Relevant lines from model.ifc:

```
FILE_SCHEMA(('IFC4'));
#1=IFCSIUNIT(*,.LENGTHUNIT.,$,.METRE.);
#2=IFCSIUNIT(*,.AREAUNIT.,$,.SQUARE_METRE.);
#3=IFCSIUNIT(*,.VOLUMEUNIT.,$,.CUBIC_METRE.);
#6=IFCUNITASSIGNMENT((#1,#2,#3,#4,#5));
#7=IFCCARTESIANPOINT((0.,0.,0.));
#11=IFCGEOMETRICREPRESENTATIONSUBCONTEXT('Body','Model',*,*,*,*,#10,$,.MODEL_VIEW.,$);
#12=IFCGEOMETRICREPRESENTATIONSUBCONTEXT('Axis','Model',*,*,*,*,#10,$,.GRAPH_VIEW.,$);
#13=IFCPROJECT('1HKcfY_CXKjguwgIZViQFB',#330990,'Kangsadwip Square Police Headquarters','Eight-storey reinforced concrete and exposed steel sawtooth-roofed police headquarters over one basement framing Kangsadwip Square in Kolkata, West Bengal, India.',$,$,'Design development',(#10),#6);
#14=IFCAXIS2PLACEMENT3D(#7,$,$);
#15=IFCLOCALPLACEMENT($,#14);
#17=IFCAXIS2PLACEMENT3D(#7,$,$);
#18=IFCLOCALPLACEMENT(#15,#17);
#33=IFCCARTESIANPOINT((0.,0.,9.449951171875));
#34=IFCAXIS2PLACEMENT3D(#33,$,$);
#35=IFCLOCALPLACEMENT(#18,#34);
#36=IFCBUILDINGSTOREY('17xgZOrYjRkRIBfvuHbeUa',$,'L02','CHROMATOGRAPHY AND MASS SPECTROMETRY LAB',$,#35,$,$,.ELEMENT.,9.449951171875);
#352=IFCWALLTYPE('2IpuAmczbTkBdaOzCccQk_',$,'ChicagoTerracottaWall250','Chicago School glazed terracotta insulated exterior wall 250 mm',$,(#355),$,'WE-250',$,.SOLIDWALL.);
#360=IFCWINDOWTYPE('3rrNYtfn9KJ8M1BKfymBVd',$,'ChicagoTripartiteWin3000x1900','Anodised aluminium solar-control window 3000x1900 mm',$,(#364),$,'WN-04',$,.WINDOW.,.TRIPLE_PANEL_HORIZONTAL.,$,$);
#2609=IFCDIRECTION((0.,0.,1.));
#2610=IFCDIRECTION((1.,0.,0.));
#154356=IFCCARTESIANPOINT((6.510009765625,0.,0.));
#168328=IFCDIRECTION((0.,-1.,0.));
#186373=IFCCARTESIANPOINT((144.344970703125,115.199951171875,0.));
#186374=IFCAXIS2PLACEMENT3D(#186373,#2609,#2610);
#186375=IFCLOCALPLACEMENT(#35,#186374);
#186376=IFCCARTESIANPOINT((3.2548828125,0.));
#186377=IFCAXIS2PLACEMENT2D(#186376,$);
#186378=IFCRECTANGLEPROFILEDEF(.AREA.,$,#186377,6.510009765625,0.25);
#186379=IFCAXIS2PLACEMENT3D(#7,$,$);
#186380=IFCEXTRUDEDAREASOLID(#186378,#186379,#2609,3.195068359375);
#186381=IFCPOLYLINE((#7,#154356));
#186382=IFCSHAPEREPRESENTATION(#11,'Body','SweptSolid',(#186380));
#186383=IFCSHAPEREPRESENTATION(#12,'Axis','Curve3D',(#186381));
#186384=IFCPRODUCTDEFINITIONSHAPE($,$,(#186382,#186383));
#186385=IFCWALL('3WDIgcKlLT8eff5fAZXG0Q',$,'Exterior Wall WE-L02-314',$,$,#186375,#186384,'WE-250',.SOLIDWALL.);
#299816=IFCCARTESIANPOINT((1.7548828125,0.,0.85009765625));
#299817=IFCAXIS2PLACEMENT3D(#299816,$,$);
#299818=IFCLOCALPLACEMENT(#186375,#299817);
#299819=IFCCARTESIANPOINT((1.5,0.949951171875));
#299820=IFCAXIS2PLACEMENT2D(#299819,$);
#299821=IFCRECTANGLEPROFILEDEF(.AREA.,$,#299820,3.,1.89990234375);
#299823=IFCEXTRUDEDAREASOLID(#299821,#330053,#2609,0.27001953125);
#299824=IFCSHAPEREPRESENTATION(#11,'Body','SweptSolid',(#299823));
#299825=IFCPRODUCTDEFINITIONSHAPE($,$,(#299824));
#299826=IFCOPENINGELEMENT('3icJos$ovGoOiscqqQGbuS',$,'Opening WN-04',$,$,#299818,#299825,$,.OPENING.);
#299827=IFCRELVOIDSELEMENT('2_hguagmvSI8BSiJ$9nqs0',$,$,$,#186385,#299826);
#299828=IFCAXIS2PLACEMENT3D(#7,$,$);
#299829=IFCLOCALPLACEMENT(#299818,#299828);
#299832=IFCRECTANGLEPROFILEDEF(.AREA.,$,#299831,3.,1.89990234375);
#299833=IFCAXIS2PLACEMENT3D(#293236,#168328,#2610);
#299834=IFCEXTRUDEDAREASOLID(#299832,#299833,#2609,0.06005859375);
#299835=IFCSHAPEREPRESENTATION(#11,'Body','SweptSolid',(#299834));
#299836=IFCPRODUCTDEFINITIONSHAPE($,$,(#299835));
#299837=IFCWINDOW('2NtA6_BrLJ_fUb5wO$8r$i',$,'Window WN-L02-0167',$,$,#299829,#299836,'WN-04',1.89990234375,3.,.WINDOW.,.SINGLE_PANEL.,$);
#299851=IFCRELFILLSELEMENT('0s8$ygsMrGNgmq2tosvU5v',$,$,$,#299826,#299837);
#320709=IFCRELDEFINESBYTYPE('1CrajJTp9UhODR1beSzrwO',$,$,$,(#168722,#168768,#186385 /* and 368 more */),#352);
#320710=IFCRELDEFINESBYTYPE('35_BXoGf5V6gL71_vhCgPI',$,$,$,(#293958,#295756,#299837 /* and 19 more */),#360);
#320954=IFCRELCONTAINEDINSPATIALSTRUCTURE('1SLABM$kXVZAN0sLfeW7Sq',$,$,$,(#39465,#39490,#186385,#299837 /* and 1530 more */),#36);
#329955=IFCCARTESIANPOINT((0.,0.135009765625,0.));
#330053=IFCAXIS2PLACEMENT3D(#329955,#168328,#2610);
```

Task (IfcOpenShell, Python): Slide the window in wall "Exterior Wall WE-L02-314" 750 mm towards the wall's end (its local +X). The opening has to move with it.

```python
import ifcopenshell
import ifcopenshell.api.geometry
import ifcopenshell.util.placement
import ifcopenshell.util.unit

model = ifcopenshell.open("model.ifc")
unit_scale = ifcopenshell.util.unit.calculate_unit_scale(model)

window = model.by_guid("2NtA6_BrLJ_fUb5wO$8r$i")
opening = window.FillsVoids[0].RelatingOpeningElement
wall = opening.VoidsElements[0].RelatingBuildingElement

wall_matrix = ifcopenshell.util.placement.get_local_placement(wall.ObjectPlacement)
shift = wall_matrix[:3, 0] * 0.75 / unit_scale
before = ifcopenshell.util.placement.get_local_placement(window.ObjectPlacement)[:3, 3].copy()

# The window is placed relative to its opening, so it follows when the opening moves.
matrix = ifcopenshell.util.placement.get_local_placement(opening.ObjectPlacement)
matrix[:3, 3] += shift
ifcopenshell.api.geometry.edit_object_placement(
    model, product=opening, matrix=matrix, is_si=False, should_transform_children=True
)

after = ifcopenshell.util.placement.get_local_placement(window.ObjectPlacement)[:3, 3]
print("window moved by", (after - before).round(3) + 0.0)

model.write("model_v2.ifc")
```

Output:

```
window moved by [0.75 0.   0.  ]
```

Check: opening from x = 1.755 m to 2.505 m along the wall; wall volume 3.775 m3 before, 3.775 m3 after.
